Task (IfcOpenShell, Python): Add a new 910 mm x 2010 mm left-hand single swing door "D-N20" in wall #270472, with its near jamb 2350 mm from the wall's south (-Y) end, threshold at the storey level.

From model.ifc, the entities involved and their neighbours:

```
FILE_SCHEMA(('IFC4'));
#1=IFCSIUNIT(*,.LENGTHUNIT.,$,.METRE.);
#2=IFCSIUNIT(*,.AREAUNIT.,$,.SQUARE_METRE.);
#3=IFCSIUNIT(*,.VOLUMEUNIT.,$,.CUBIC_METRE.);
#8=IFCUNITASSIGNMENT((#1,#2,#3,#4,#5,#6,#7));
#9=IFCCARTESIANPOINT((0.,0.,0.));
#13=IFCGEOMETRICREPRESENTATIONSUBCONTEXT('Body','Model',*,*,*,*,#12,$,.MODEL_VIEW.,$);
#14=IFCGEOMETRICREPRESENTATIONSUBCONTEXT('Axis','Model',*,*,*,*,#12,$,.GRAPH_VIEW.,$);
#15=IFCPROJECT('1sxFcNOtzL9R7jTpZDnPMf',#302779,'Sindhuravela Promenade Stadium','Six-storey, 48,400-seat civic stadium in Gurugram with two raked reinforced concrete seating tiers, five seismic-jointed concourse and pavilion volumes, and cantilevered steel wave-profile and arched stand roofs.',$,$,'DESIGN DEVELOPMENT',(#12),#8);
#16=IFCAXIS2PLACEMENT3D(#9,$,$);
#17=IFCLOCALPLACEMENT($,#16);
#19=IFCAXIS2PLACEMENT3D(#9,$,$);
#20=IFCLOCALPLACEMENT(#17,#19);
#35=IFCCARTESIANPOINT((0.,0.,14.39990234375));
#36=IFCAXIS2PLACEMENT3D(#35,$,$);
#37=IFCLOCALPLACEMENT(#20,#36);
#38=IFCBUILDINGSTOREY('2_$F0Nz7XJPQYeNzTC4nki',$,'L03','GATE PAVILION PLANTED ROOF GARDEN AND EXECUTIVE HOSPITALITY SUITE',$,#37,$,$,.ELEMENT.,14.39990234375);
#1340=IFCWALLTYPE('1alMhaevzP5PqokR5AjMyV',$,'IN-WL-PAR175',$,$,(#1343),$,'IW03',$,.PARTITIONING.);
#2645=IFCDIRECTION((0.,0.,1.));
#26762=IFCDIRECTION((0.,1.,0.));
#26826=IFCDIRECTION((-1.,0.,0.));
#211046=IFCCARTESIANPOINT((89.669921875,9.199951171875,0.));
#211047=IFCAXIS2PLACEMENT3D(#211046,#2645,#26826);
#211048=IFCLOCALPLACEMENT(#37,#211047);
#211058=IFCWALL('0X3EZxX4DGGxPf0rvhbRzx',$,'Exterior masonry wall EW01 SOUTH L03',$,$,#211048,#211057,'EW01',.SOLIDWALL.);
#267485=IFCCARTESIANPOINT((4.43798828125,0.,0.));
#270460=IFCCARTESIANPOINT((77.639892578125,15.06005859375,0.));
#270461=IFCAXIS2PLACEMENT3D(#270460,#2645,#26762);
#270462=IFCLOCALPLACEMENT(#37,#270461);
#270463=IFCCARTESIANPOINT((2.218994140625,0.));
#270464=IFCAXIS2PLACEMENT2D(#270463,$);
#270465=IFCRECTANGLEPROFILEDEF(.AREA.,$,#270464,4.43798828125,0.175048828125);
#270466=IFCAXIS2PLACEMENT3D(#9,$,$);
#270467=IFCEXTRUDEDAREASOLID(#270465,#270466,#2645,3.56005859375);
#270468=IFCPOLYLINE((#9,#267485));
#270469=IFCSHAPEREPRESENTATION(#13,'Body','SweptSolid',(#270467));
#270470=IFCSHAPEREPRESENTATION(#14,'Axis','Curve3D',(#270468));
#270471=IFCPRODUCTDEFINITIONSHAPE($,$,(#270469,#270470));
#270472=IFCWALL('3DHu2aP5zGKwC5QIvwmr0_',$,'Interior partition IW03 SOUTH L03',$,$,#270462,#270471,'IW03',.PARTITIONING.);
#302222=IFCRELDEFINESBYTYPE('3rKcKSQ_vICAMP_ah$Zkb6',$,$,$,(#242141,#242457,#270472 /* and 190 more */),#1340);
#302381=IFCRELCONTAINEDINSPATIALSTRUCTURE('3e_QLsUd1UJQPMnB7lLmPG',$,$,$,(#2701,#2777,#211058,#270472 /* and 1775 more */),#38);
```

```python
import numpy as np
import ifcopenshell
import ifcopenshell.api.feature
import ifcopenshell.api.geometry
import ifcopenshell.api.root
import ifcopenshell.api.spatial
import ifcopenshell.geom
import ifcopenshell.util.element
import ifcopenshell.util.placement
import ifcopenshell.util.representation
import ifcopenshell.util.shape
import ifcopenshell.util.unit

model = ifcopenshell.open("model.ifc")
unit_scale = ifcopenshell.util.unit.calculate_unit_scale(model)
settings = ifcopenshell.geom.settings()


def volume(element):
    """Net volume in cubic metres, openings subtracted."""
    shape = ifcopenshell.geom.create_shape(settings, element)
    return ifcopenshell.util.shape.get_volume(shape.geometry)


wall = model.by_guid("3DHu2aP5zGKwC5QIvwmr0_")
storey = ifcopenshell.util.element.get_container(wall, ifc_class="IfcBuildingStorey")
context = ifcopenshell.util.representation.get_context(model, "Model", "Body", "MODEL_VIEW")
before = volume(wall)

width, height, from_end, sill = 0.91, 2.01, 2.35, 0.0  # metres

# The wall runs along its own X axis, and the end named is its -X end.
wall_shape = ifcopenshell.geom.create_shape(settings, wall)
x, y, z = ifcopenshell.util.shape.get_vertices(wall_shape.geometry).T
start = x.min() + from_end
face, thickness = float(y.min()), float(y.max() - y.min())
wall_matrix = ifcopenshell.util.placement.get_local_placement(wall.ObjectPlacement)
level = ifcopenshell.util.placement.get_local_placement(storey.ObjectPlacement)[2, 3]


def in_wall(x, y):
    """Placement at x, y metres in the wall's axes, at sill height."""
    matrix = wall_matrix.copy()
    matrix[:, 3] = wall_matrix @ np.array([x / unit_scale, y / unit_scale, 0.0, 1.0])
    matrix[2, 3] = level + sill / unit_scale
    return matrix


# Opening: a box that overshoots both wall faces by 50 mm.
opening = ifcopenshell.api.root.create_entity(model, ifc_class="IfcOpeningElement", predefined_type="OPENING")
box = ifcopenshell.api.geometry.add_wall_representation(
    model, context=context, length=width, height=height, thickness=thickness + 0.1
)
ifcopenshell.api.geometry.assign_representation(model, product=opening, representation=box)
ifcopenshell.api.geometry.edit_object_placement(model, product=opening, matrix=in_wall(start, face - 0.05), is_si=False)
ifcopenshell.api.feature.add_feature(model, feature=opening, element=wall)

door = ifcopenshell.api.root.create_entity(model, ifc_class="IfcDoor", name="D-N20", predefined_type="DOOR")
door.OverallWidth, door.OverallHeight = width / unit_scale, height / unit_scale
door.OperationType = "SINGLE_SWING_LEFT"
body = ifcopenshell.api.geometry.add_door_representation(
    model,
    context=context,
    overall_width=door.OverallWidth,
    overall_height=door.OverallHeight,
    operation_type="SINGLE_SWING_LEFT",
    lining_properties={"LiningDepth": thickness / unit_scale, "ThresholdDepth": thickness / unit_scale},
)
ifcopenshell.api.geometry.assign_representation(model, product=door, representation=body)
ifcopenshell.api.spatial.assign_container(model, products=[door], relating_structure=storey)
ifcopenshell.api.feature.add_filling(model, opening=opening, element=door)

# The lining spans the wall, so the door starts at the wall face.
ifcopenshell.api.geometry.edit_object_placement(model, product=door, matrix=in_wall(start, face), is_si=False)

after = volume(wall)

print(f"wall volume {before:.3f} -> {after:.3f} m3")

model.write("model_rev.ifc")
```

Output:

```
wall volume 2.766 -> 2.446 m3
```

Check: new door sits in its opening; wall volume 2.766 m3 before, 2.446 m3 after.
